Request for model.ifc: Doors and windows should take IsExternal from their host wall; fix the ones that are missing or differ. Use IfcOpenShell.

First a look at what the model holds.

```python
import ifcopenshell
import ifcopenshell.util.element

model = ifcopenshell.open("model.ifc")
print(model.schema)
seen = {}
for e in model.by_type("IfcDoor") + model.by_type("IfcWindow"):
    if not e.FillsVoids:
        continue
    host = e.FillsVoids[0].RelatingOpeningElement.VoidsElements[0].RelatingBuildingElement
    own = ifcopenshell.util.element.get_pset(e, f"Pset_{e.is_a()[3:].removesuffix('StandardCase')}Common", "IsExternal")
    wall = ifcopenshell.util.element.get_pset(host, "Pset_WallCommon", "IsExternal")
    seen[e.is_a(), own, wall] = seen.get((e.is_a(), own, wall), 0) + 1
for (cls, own, wall), count in sorted(seen.items(), key=str):
    print(count, cls, "IsExternal:", own, "| host wall:", wall)
```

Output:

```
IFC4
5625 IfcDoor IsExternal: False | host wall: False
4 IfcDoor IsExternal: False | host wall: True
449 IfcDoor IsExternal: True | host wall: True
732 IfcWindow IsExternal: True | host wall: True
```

```python
import ifcopenshell
import ifcopenshell.api.pset
import ifcopenshell.util.element

model = ifcopenshell.open("model.ifc")

count = 0
for ifc_class, pset_name in (("IfcDoor", "Pset_DoorCommon"), ("IfcWindow", "Pset_WindowCommon")):
    for e in model.by_type(ifc_class):
        if not e.FillsVoids:
            continue
        host = e.FillsVoids[0].RelatingOpeningElement.VoidsElements[0].RelatingBuildingElement
        external = ifcopenshell.util.element.get_pset(host, "Pset_WallCommon", "IsExternal")
        if external is None or ifcopenshell.util.element.get_pset(e, pset_name, "IsExternal") == external:
            continue
        found = ifcopenshell.util.element.get_pset(e, pset_name, should_inherit=False)
        if found:
            pset = model.by_id(found["id"])
            if len(ifcopenshell.util.element.get_elements_by_pset(pset)) > 1:
                pset = ifcopenshell.api.pset.unshare_pset(model, products=[e], pset=pset)[0]
        else:
            pset = ifcopenshell.api.pset.add_pset(model, product=e, name=pset_name)
        ifcopenshell.api.pset.edit_pset(model, pset=pset, properties={"IsExternal": external})
        count += 1

print(count, "updated")

model.write("model_updated.ifc")
```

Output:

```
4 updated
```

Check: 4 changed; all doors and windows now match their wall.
